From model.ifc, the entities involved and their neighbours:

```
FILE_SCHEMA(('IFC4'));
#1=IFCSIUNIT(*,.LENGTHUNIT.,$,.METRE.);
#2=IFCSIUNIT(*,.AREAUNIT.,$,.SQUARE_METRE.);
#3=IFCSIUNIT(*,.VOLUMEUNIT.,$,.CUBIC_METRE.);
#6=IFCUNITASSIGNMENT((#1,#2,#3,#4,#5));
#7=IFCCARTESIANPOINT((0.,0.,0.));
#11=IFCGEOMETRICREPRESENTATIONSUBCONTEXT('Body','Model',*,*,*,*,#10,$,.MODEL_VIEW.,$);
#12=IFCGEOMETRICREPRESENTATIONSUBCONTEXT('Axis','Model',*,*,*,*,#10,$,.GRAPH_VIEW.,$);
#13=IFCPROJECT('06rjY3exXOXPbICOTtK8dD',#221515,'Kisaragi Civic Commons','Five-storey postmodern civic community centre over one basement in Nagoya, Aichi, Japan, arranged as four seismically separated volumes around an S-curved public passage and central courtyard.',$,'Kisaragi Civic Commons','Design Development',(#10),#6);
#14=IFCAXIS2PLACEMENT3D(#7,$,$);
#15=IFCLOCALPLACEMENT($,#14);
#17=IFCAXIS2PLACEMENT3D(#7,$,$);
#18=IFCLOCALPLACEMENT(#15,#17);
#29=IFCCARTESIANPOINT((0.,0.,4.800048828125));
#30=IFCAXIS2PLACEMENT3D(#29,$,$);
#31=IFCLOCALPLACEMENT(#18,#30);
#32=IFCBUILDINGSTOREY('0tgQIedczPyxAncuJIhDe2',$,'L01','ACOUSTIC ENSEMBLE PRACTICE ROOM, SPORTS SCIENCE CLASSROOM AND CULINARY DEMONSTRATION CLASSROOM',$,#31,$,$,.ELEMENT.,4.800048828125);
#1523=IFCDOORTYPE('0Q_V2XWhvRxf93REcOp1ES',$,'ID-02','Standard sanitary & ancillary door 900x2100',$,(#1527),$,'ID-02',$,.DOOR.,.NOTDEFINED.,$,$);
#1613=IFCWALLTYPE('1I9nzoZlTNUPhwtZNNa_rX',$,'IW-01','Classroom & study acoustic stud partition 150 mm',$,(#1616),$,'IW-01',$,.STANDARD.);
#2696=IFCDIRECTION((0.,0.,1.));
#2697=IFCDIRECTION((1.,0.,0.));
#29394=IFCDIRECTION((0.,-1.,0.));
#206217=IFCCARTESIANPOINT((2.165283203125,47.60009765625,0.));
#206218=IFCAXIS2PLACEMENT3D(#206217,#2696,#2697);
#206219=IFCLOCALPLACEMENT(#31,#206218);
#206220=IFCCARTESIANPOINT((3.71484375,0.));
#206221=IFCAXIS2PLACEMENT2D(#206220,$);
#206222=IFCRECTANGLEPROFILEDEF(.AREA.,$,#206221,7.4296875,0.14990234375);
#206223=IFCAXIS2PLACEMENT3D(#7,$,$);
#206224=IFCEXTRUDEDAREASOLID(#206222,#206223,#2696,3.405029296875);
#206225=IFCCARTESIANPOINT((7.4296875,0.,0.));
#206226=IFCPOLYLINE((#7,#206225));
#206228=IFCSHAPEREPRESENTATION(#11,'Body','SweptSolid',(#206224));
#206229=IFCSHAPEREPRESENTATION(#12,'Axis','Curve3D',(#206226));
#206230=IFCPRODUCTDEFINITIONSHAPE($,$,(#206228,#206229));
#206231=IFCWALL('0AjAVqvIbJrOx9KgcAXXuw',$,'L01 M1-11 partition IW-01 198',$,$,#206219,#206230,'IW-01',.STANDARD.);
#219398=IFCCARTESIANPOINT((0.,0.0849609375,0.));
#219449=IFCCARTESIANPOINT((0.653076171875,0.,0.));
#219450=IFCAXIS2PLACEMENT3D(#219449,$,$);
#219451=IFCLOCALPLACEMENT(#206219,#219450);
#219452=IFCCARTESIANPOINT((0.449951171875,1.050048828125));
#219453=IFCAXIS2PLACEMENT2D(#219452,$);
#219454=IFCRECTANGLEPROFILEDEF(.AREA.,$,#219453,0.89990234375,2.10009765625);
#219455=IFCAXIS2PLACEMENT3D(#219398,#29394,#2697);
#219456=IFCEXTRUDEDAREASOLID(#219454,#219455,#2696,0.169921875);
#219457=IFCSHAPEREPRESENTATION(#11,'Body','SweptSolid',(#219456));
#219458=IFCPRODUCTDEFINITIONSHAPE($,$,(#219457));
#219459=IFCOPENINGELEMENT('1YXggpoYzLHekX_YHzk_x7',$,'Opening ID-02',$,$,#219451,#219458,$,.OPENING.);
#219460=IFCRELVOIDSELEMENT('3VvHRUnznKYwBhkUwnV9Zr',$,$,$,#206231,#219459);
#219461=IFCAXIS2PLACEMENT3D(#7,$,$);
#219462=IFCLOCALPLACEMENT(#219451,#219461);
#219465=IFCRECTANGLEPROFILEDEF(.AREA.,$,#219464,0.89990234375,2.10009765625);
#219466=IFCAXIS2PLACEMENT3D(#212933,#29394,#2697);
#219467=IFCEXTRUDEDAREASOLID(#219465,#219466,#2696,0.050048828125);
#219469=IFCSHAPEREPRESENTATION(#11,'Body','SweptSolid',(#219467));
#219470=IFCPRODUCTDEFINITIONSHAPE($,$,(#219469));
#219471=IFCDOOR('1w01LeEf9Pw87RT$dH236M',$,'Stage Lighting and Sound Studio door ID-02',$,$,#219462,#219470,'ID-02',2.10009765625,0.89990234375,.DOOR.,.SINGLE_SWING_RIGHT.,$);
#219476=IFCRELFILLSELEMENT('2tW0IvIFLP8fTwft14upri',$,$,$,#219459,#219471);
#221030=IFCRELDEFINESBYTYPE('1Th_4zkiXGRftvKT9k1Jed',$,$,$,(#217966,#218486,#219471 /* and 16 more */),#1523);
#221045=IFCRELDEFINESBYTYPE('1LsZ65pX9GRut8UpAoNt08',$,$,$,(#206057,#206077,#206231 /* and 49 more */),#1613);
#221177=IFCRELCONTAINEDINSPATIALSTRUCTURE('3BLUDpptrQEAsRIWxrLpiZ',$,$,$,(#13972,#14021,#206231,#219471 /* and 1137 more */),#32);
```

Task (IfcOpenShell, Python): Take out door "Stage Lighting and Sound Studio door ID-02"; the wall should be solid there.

```python
import ifcopenshell
import ifcopenshell.api.feature
import ifcopenshell.api.root
import ifcopenshell.geom
import ifcopenshell.util.shape

model = ifcopenshell.open("model.ifc")
settings = ifcopenshell.geom.settings()


def volume(element):
    """Net volume in cubic metres, openings subtracted."""
    shape = ifcopenshell.geom.create_shape(settings, element)
    return ifcopenshell.util.shape.get_volume(shape.geometry)


door = model.by_id(219471)
opening = door.FillsVoids[0].RelatingOpeningElement
wall = opening.VoidsElements[0].RelatingBuildingElement
before = volume(wall)

ifcopenshell.api.root.remove_product(model, product=door)
ifcopenshell.api.feature.remove_feature(model, feature=opening)

after = volume(wall)

print(f"wall volume {before:.3f} -> {after:.3f} m3")

model.write("model_edited.ifc")
```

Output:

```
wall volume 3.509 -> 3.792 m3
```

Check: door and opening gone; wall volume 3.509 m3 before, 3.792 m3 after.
